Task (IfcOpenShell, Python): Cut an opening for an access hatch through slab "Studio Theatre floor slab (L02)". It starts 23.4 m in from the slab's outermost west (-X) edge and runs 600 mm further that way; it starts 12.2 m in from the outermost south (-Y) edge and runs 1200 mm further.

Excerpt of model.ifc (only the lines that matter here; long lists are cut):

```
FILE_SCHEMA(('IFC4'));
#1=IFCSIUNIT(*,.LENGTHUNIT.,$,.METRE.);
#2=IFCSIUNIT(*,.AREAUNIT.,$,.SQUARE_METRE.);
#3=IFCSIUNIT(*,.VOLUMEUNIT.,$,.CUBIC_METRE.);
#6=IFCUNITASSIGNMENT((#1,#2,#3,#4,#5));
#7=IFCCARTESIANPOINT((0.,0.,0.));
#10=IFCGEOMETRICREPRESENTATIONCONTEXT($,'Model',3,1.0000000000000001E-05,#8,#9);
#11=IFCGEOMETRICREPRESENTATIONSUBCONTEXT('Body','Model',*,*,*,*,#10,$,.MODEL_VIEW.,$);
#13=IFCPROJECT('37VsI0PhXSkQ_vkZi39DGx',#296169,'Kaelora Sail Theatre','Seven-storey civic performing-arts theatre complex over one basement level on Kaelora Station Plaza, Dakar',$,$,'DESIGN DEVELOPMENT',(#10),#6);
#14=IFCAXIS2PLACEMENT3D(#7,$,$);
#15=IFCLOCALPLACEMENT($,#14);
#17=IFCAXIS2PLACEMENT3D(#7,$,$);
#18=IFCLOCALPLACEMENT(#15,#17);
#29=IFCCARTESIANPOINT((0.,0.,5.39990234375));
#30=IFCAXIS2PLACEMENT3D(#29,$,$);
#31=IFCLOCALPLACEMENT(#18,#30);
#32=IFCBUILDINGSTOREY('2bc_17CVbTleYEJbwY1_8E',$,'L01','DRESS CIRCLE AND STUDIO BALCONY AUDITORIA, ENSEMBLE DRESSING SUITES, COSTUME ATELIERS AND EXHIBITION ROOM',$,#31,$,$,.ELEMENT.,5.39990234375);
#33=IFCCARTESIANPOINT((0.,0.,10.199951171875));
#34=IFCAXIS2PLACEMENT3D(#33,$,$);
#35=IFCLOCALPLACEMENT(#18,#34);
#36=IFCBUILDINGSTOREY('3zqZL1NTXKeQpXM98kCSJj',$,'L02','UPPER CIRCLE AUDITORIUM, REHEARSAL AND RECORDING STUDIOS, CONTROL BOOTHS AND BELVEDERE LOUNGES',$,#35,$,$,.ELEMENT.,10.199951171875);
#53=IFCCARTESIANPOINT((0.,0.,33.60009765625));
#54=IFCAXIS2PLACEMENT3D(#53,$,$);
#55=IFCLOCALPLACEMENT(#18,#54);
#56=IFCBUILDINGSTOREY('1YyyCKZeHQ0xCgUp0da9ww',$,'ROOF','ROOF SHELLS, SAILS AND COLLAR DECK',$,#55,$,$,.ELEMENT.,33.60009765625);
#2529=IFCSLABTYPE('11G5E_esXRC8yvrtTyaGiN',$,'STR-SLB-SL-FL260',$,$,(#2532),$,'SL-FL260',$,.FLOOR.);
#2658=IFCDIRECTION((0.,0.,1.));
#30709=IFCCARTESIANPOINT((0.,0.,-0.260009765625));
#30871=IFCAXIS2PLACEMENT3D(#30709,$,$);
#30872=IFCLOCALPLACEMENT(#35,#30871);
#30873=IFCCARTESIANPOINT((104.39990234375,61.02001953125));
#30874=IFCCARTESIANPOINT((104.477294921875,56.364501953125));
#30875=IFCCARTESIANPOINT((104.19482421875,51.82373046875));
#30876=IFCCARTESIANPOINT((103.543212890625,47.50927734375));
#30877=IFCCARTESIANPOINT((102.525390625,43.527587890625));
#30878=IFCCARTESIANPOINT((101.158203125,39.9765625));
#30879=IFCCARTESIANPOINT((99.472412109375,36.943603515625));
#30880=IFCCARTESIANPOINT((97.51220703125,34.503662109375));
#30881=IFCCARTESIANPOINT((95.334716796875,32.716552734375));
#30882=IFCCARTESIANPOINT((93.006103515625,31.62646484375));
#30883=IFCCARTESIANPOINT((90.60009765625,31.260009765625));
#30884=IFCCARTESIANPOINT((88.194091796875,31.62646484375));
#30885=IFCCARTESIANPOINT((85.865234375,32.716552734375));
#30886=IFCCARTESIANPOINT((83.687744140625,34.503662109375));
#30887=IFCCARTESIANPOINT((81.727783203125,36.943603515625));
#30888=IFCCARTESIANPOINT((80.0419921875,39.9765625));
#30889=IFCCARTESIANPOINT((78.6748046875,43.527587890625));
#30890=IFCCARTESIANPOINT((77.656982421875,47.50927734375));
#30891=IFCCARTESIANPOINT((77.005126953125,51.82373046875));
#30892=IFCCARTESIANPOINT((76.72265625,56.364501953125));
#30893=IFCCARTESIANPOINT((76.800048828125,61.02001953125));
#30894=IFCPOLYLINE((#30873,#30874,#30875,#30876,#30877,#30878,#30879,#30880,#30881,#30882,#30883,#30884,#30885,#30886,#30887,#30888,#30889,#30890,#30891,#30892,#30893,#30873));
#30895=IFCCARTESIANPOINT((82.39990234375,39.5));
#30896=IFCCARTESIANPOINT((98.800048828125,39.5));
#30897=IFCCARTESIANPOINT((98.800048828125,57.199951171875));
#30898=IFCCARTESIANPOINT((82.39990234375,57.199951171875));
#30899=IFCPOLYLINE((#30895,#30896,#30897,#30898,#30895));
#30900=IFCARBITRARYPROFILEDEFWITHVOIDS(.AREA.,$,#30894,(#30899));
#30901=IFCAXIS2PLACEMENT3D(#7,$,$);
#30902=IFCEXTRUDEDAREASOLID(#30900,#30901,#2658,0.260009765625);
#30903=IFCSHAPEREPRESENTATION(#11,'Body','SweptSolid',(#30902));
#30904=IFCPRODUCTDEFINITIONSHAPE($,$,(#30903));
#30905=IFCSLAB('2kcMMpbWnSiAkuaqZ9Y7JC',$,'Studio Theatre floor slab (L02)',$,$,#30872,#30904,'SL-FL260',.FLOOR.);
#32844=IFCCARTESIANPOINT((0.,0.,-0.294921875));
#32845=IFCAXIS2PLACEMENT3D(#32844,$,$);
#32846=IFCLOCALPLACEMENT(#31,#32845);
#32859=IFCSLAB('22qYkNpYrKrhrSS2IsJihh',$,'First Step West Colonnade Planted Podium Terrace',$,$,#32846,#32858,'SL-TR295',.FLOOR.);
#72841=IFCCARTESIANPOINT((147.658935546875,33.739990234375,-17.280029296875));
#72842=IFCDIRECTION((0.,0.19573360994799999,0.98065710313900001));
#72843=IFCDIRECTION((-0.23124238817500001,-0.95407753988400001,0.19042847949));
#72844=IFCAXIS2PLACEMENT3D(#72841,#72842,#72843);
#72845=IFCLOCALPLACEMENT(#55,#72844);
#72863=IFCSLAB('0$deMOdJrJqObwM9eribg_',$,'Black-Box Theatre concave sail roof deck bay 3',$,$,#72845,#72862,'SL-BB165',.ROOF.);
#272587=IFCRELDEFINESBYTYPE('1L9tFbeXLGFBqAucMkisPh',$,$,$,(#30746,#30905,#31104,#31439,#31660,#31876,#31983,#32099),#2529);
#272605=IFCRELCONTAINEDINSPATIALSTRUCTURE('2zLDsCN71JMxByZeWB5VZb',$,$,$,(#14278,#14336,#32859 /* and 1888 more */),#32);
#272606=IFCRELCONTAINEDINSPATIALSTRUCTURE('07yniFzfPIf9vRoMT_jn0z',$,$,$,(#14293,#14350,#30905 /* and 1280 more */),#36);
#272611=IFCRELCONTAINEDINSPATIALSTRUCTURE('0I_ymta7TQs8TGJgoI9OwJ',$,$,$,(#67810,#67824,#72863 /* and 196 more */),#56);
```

```python
import numpy as np
import ifcopenshell
import ifcopenshell.api.feature
import ifcopenshell.api.geometry
import ifcopenshell.api.root
import ifcopenshell.geom
import ifcopenshell.util.placement
import ifcopenshell.util.representation
import ifcopenshell.util.shape
import ifcopenshell.util.unit

model = ifcopenshell.open("model.ifc")
unit_scale = ifcopenshell.util.unit.calculate_unit_scale(model)
settings = ifcopenshell.geom.settings()


def volume(element):
    """Net volume in cubic metres, openings subtracted."""
    shape = ifcopenshell.geom.create_shape(settings, element)
    return ifcopenshell.util.shape.get_volume(shape.geometry)


slab = model.by_guid("2kcMMpbWnSiAkuaqZ9Y7JC")
before = volume(slab)

# Extent in the slab's own axes, in metres. The edges named are its -X and -Y sides.
slab_shape = ifcopenshell.geom.create_shape(settings, slab)
vertices = ifcopenshell.util.shape.get_vertices(slab_shape.geometry)
x_min, y_min, bottom = vertices.min(axis=0)
top = vertices[:, 2].max()

opening = ifcopenshell.api.root.create_entity(model, ifc_class="IfcOpeningElement", name="Access hatch opening", predefined_type="OPENING")
context = ifcopenshell.util.representation.get_context(model, "Model", "Body", "MODEL_VIEW")
width, depth = 0.6, 1.2
outline = [(0.0, 0.0), (width, 0.0), (width, depth), (0.0, depth), (0.0, 0.0)]
# Overshoot both faces by 50 mm so the cut is clean.
shape = ifcopenshell.api.geometry.add_slab_representation(
    model, context=context, depth=top - bottom + 0.1, polyline=outline
)
ifcopenshell.api.geometry.assign_representation(model, product=opening, representation=shape)

matrix = ifcopenshell.util.placement.get_local_placement(slab.ObjectPlacement)
matrix[:, 3] = matrix @ np.append(np.array([x_min + 23.4, y_min + 12.2, bottom - 0.05]) / unit_scale, 1.0)
ifcopenshell.api.geometry.edit_object_placement(model, product=opening, matrix=matrix, is_si=False)
ifcopenshell.api.feature.add_feature(model, feature=opening, element=slab)

after = volume(slab)

print(f"slab volume {before:.3f} -> {after:.3f} m3")

model.write("model_updated.ifc")
```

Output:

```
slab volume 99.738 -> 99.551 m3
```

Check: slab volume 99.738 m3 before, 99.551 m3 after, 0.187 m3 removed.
